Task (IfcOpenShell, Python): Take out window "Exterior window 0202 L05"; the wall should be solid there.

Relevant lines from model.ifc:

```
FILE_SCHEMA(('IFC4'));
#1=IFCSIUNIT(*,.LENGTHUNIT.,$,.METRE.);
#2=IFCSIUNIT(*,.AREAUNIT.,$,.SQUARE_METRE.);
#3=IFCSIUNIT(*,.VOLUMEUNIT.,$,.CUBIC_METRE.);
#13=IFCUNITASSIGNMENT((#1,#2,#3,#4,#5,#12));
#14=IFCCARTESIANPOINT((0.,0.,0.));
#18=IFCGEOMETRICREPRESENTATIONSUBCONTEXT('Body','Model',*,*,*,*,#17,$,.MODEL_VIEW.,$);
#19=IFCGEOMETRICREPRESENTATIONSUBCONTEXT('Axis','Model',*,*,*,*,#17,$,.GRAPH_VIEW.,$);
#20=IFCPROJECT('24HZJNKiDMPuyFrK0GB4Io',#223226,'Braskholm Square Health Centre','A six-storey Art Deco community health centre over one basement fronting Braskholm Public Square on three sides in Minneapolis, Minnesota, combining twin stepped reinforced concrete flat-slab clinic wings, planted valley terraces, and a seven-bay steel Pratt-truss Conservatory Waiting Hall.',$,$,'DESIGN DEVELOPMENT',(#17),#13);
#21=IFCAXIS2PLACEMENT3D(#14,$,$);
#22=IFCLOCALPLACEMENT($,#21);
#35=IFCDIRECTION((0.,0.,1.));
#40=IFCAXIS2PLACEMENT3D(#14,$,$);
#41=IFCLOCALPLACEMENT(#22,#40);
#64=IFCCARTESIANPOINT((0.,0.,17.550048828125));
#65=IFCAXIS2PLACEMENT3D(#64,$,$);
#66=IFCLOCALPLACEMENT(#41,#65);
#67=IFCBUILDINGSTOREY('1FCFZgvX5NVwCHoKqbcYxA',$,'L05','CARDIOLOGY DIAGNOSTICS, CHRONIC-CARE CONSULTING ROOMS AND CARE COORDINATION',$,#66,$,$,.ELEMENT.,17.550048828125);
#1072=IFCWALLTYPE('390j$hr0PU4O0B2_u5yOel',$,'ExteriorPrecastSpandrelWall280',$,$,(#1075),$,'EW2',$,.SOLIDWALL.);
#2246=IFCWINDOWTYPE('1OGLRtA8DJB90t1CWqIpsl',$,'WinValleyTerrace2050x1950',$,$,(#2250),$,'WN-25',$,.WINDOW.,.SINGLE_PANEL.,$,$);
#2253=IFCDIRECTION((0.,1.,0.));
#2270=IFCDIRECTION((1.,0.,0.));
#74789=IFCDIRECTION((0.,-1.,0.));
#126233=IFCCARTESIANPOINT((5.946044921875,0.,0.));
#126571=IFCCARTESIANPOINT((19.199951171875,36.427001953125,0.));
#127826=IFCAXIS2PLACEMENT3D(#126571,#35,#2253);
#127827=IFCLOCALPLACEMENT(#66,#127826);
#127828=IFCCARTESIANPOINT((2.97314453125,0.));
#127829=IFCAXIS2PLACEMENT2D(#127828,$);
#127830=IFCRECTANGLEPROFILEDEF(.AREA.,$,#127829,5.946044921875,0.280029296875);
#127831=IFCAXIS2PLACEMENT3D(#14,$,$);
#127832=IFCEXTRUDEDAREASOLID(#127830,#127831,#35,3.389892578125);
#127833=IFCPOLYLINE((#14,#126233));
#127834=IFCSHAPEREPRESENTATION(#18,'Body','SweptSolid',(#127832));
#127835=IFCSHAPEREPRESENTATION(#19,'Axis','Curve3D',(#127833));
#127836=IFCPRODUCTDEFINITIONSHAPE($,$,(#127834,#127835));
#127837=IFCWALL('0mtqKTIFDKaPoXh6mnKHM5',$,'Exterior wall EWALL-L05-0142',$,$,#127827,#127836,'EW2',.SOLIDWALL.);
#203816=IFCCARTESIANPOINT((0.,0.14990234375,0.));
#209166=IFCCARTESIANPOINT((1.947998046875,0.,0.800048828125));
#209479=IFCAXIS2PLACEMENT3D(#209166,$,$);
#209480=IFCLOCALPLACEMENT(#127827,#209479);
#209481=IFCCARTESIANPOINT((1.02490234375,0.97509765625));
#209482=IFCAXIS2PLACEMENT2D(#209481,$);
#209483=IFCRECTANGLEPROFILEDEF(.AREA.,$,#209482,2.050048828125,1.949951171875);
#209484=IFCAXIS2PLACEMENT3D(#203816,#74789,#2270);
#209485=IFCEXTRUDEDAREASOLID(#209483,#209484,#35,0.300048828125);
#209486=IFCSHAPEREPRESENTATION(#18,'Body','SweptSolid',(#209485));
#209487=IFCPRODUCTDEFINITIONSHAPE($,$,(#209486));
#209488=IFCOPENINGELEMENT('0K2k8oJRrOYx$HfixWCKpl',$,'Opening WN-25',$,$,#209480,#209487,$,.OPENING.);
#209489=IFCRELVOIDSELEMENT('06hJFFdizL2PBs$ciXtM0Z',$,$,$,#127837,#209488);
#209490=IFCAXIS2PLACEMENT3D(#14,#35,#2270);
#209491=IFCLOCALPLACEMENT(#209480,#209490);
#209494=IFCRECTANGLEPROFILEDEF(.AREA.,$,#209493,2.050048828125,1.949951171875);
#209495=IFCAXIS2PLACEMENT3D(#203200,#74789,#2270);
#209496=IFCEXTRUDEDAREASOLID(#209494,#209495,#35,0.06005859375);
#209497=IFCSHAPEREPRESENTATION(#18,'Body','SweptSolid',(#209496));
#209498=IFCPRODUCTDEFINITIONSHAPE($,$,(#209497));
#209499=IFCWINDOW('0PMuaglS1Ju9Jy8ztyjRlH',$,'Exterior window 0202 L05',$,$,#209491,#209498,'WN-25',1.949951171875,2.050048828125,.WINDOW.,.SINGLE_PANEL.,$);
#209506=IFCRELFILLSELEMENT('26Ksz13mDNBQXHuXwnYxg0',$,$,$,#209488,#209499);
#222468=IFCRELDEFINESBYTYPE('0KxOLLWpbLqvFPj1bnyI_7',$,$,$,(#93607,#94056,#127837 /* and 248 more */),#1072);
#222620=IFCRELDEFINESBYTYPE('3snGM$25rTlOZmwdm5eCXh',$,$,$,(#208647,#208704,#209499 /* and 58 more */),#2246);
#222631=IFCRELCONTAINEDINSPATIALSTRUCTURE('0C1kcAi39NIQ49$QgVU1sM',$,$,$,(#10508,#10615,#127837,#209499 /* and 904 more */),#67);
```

```python
import ifcopenshell
import ifcopenshell.api.feature
import ifcopenshell.api.root
import ifcopenshell.geom
import ifcopenshell.util.shape

model = ifcopenshell.open("model.ifc")
settings = ifcopenshell.geom.settings()


def volume(element):
    """Net volume in cubic metres, openings subtracted."""
    shape = ifcopenshell.geom.create_shape(settings, element)
    return ifcopenshell.util.shape.get_volume(shape.geometry)


window = model.by_guid("0PMuaglS1Ju9Jy8ztyjRlH")
opening = window.FillsVoids[0].RelatingOpeningElement
wall = opening.VoidsElements[0].RelatingBuildingElement
before = volume(wall)

ifcopenshell.api.root.remove_product(model, product=window)
ifcopenshell.api.feature.remove_feature(model, feature=opening)

after = volume(wall)

print(f"wall volume {before:.3f} -> {after:.3f} m3")

model.write("model_edited.ifc")
```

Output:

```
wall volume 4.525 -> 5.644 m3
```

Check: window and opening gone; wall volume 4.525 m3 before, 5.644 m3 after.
